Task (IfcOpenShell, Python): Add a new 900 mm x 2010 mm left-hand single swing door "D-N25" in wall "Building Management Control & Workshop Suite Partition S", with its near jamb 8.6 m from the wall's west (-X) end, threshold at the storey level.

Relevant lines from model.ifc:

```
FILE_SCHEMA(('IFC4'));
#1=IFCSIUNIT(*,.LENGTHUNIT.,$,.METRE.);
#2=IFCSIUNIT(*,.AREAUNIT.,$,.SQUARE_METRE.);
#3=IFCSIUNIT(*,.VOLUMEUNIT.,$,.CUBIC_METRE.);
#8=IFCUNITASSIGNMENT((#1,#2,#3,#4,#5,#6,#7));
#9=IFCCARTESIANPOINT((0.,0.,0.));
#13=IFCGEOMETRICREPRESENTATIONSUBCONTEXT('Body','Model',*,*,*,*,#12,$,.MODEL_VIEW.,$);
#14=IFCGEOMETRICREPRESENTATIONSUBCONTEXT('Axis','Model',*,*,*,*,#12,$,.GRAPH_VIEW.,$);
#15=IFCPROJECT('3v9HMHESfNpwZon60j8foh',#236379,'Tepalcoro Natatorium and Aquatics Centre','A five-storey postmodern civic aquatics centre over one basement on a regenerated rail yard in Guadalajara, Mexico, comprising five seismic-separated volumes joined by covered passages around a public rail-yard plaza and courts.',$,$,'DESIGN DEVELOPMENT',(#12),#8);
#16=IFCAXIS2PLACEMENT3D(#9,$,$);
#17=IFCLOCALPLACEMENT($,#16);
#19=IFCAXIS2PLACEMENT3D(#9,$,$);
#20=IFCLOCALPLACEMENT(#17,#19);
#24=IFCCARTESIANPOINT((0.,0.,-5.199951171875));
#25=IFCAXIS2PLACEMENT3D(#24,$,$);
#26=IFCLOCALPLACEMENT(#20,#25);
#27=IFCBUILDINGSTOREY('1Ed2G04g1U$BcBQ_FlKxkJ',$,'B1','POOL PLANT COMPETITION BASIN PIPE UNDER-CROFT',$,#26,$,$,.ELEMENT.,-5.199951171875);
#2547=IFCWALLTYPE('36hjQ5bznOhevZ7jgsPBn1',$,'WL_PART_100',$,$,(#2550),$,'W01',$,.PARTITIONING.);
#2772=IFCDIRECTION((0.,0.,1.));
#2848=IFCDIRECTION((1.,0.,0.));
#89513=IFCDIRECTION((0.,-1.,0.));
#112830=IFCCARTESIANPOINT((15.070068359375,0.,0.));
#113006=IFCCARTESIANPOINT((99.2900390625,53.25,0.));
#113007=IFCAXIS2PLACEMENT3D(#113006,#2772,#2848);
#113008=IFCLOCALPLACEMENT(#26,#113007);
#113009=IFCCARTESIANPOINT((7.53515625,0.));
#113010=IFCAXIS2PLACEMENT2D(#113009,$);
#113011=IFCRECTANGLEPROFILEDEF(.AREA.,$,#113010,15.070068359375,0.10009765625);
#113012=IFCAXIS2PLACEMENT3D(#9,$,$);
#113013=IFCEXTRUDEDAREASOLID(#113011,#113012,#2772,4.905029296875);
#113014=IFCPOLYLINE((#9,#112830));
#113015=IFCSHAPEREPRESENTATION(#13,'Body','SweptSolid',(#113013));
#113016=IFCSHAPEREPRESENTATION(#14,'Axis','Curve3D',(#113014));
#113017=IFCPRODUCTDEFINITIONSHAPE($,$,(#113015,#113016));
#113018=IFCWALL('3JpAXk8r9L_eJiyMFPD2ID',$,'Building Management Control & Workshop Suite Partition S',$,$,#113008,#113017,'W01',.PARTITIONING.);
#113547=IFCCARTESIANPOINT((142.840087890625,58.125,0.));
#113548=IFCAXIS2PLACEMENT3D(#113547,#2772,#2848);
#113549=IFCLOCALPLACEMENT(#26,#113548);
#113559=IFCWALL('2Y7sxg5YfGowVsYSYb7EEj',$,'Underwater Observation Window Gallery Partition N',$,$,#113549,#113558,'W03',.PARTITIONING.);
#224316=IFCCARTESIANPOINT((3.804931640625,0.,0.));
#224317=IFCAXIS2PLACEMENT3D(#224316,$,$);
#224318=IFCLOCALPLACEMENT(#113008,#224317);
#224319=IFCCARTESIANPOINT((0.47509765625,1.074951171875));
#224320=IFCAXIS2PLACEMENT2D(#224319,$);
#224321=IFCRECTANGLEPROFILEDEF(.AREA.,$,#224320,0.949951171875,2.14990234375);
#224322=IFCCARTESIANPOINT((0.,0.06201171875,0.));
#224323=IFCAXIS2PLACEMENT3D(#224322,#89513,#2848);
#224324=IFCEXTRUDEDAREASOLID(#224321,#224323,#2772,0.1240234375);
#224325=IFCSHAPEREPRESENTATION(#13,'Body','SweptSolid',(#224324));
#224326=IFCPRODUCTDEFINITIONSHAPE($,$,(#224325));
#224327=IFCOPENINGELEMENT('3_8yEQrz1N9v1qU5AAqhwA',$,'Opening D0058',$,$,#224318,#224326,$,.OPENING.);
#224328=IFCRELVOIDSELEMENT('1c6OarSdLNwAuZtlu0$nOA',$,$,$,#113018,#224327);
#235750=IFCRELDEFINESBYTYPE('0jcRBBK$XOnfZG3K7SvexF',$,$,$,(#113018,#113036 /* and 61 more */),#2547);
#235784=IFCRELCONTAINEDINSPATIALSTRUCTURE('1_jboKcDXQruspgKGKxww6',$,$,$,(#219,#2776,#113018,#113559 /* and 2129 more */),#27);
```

```python
import numpy as np
import ifcopenshell
import ifcopenshell.api.feature
import ifcopenshell.api.geometry
import ifcopenshell.api.root
import ifcopenshell.api.spatial
import ifcopenshell.geom
import ifcopenshell.util.element
import ifcopenshell.util.placement
import ifcopenshell.util.representation
import ifcopenshell.util.shape
import ifcopenshell.util.unit

model = ifcopenshell.open("model.ifc")
unit_scale = ifcopenshell.util.unit.calculate_unit_scale(model)
settings = ifcopenshell.geom.settings()


def volume(element):
    """Net volume in cubic metres, openings subtracted."""
    shape = ifcopenshell.geom.create_shape(settings, element)
    return ifcopenshell.util.shape.get_volume(shape.geometry)


wall = model.by_guid("3JpAXk8r9L_eJiyMFPD2ID")
storey = ifcopenshell.util.element.get_container(wall, ifc_class="IfcBuildingStorey")
context = ifcopenshell.util.representation.get_context(model, "Model", "Body", "MODEL_VIEW")
before = volume(wall)

width, height, from_end, sill = 0.9, 2.01, 8.6, 0.0  # metres

# The wall runs along its own X axis, and the end named is its -X end.
wall_shape = ifcopenshell.geom.create_shape(settings, wall)
x, y, z = ifcopenshell.util.shape.get_vertices(wall_shape.geometry).T
start = x.min() + from_end
face, thickness = float(y.min()), float(y.max() - y.min())
wall_matrix = ifcopenshell.util.placement.get_local_placement(wall.ObjectPlacement)
level = ifcopenshell.util.placement.get_local_placement(storey.ObjectPlacement)[2, 3]


def in_wall(x, y):
    """Placement at x, y metres in the wall's axes, at sill height."""
    matrix = wall_matrix.copy()
    matrix[:, 3] = wall_matrix @ np.array([x / unit_scale, y / unit_scale, 0.0, 1.0])
    matrix[2, 3] = level + sill / unit_scale
    return matrix


# Opening: a box that overshoots both wall faces by 50 mm.
opening = ifcopenshell.api.root.create_entity(model, ifc_class="IfcOpeningElement", predefined_type="OPENING")
box = ifcopenshell.api.geometry.add_wall_representation(
    model, context=context, length=width, height=height, thickness=thickness + 0.1
)
ifcopenshell.api.geometry.assign_representation(model, product=opening, representation=box)
ifcopenshell.api.geometry.edit_object_placement(model, product=opening, matrix=in_wall(start, face - 0.05), is_si=False)
ifcopenshell.api.feature.add_feature(model, feature=opening, element=wall)

door = ifcopenshell.api.root.create_entity(model, ifc_class="IfcDoor", name="D-N25", predefined_type="DOOR")
door.OverallWidth, door.OverallHeight = width / unit_scale, height / unit_scale
door.OperationType = "SINGLE_SWING_LEFT"
body = ifcopenshell.api.geometry.add_door_representation(
    model,
    context=context,
    overall_width=door.OverallWidth,
    overall_height=door.OverallHeight,
    operation_type="SINGLE_SWING_LEFT",
    lining_properties={"LiningDepth": thickness / unit_scale, "ThresholdDepth": thickness / unit_scale},
)
ifcopenshell.api.geometry.assign_representation(model, product=door, representation=body)
ifcopenshell.api.spatial.assign_container(model, products=[door], relating_structure=storey)
ifcopenshell.api.feature.add_filling(model, opening=opening, element=door)

# The lining spans the wall, so the door starts at the wall face.
ifcopenshell.api.geometry.edit_object_placement(model, product=door, matrix=in_wall(start, face), is_si=False)

after = volume(wall)

print(f"wall volume {before:.3f} -> {after:.3f} m3")

model.write("model_rev.ifc")
```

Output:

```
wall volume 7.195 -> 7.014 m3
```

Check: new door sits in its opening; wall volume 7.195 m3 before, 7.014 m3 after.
